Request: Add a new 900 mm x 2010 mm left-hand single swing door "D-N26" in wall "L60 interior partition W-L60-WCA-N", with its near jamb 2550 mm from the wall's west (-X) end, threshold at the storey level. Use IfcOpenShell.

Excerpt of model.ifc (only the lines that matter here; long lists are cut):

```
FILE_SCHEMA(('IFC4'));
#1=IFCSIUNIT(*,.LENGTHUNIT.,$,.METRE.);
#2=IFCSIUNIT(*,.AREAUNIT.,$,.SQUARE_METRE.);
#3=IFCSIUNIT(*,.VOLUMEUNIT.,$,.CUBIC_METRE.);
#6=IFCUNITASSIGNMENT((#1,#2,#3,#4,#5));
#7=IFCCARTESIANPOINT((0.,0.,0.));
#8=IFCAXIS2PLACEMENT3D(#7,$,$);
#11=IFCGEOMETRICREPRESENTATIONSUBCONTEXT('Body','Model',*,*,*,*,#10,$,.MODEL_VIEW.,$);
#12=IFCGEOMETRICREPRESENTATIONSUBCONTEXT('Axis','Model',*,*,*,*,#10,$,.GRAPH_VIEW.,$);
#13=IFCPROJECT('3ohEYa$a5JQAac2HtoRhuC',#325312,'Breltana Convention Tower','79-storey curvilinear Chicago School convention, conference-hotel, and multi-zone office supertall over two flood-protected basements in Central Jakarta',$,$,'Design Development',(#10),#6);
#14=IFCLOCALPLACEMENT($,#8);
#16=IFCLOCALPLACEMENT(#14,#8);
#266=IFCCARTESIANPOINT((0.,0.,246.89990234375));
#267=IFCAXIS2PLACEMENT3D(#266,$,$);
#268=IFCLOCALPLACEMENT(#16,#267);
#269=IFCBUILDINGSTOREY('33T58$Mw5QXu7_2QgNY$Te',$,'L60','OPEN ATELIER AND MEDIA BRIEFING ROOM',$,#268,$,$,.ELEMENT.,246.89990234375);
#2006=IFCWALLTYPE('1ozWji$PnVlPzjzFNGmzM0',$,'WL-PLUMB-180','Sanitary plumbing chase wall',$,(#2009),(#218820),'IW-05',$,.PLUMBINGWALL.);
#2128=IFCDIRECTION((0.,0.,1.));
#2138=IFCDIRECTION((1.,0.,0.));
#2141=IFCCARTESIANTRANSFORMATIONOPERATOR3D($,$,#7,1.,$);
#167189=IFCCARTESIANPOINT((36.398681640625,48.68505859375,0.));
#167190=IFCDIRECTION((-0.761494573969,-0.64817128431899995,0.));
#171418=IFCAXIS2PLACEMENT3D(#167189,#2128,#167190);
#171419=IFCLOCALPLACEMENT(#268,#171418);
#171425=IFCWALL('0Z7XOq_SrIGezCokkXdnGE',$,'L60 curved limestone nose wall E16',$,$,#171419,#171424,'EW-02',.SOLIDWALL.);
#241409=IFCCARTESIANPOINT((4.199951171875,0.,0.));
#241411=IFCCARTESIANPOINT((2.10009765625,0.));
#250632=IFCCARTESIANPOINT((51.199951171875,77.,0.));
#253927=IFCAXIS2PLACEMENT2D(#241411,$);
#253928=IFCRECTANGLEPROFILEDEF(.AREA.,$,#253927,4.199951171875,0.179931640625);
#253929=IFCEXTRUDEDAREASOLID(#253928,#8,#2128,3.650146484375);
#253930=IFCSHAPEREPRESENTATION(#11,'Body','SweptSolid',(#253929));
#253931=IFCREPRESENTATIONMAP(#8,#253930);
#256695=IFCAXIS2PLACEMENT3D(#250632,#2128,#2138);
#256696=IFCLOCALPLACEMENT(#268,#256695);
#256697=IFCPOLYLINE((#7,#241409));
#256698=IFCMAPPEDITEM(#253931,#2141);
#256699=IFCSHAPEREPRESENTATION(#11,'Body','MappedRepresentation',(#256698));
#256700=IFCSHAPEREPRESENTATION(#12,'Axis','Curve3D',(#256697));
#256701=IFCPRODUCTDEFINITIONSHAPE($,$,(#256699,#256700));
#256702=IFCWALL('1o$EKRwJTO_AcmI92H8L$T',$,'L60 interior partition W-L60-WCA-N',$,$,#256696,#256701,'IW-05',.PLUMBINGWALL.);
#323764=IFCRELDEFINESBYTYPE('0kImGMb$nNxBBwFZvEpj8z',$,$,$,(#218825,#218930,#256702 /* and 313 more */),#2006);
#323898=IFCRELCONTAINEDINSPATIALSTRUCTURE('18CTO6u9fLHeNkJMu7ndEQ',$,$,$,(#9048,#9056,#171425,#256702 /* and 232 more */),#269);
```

```python
import numpy as np
import ifcopenshell
import ifcopenshell.api.feature
import ifcopenshell.api.geometry
import ifcopenshell.api.root
import ifcopenshell.api.spatial
import ifcopenshell.geom
import ifcopenshell.util.element
import ifcopenshell.util.placement
import ifcopenshell.util.representation
import ifcopenshell.util.shape
import ifcopenshell.util.unit

model = ifcopenshell.open("model.ifc")
unit_scale = ifcopenshell.util.unit.calculate_unit_scale(model)
settings = ifcopenshell.geom.settings()


def volume(element):
    """Net volume in cubic metres, openings subtracted."""
    shape = ifcopenshell.geom.create_shape(settings, element)
    return ifcopenshell.util.shape.get_volume(shape.geometry)


wall = model.by_guid("1o$EKRwJTO_AcmI92H8L$T")
storey = ifcopenshell.util.element.get_container(wall, ifc_class="IfcBuildingStorey")
context = ifcopenshell.util.representation.get_context(model, "Model", "Body", "MODEL_VIEW")
before = volume(wall)

width, height, from_end, sill = 0.9, 2.01, 2.55, 0.0  # metres

# The wall runs along its own X axis, and the end named is its -X end.
wall_shape = ifcopenshell.geom.create_shape(settings, wall)
x, y, z = ifcopenshell.util.shape.get_vertices(wall_shape.geometry).T
start = x.min() + from_end
face, thickness = float(y.min()), float(y.max() - y.min())
wall_matrix = ifcopenshell.util.placement.get_local_placement(wall.ObjectPlacement)
level = ifcopenshell.util.placement.get_local_placement(storey.ObjectPlacement)[2, 3]


def in_wall(x, y):
    """Placement at x, y metres in the wall's axes, at sill height."""
    matrix = wall_matrix.copy()
    matrix[:, 3] = wall_matrix @ np.array([x / unit_scale, y / unit_scale, 0.0, 1.0])
    matrix[2, 3] = level + sill / unit_scale
    return matrix


# Opening: a box that overshoots both wall faces by 50 mm.
opening = ifcopenshell.api.root.create_entity(model, ifc_class="IfcOpeningElement", predefined_type="OPENING")
box = ifcopenshell.api.geometry.add_wall_representation(
    model, context=context, length=width, height=height, thickness=thickness + 0.1
)
ifcopenshell.api.geometry.assign_representation(model, product=opening, representation=box)
ifcopenshell.api.geometry.edit_object_placement(model, product=opening, matrix=in_wall(start, face - 0.05), is_si=False)
ifcopenshell.api.feature.add_feature(model, feature=opening, element=wall)

door = ifcopenshell.api.root.create_entity(model, ifc_class="IfcDoor", name="D-N26", predefined_type="DOOR")
door.OverallWidth, door.OverallHeight = width / unit_scale, height / unit_scale
door.OperationType = "SINGLE_SWING_LEFT"
body = ifcopenshell.api.geometry.add_door_representation(
    model,
    context=context,
    overall_width=door.OverallWidth,
    overall_height=door.OverallHeight,
    operation_type="SINGLE_SWING_LEFT",
    lining_properties={"LiningDepth": thickness / unit_scale, "ThresholdDepth": thickness / unit_scale},
)
ifcopenshell.api.geometry.assign_representation(model, product=door, representation=body)
ifcopenshell.api.spatial.assign_container(model, products=[door], relating_structure=storey)
ifcopenshell.api.feature.add_filling(model, opening=opening, element=door)

# The lining spans the wall, so the door starts at the wall face.
ifcopenshell.api.geometry.edit_object_placement(model, product=door, matrix=in_wall(start, face), is_si=False)

after = volume(wall)

print(f"wall volume {before:.3f} -> {after:.3f} m3")

model.write("model_updated.ifc")
```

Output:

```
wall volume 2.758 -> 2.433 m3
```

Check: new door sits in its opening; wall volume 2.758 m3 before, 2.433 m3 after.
